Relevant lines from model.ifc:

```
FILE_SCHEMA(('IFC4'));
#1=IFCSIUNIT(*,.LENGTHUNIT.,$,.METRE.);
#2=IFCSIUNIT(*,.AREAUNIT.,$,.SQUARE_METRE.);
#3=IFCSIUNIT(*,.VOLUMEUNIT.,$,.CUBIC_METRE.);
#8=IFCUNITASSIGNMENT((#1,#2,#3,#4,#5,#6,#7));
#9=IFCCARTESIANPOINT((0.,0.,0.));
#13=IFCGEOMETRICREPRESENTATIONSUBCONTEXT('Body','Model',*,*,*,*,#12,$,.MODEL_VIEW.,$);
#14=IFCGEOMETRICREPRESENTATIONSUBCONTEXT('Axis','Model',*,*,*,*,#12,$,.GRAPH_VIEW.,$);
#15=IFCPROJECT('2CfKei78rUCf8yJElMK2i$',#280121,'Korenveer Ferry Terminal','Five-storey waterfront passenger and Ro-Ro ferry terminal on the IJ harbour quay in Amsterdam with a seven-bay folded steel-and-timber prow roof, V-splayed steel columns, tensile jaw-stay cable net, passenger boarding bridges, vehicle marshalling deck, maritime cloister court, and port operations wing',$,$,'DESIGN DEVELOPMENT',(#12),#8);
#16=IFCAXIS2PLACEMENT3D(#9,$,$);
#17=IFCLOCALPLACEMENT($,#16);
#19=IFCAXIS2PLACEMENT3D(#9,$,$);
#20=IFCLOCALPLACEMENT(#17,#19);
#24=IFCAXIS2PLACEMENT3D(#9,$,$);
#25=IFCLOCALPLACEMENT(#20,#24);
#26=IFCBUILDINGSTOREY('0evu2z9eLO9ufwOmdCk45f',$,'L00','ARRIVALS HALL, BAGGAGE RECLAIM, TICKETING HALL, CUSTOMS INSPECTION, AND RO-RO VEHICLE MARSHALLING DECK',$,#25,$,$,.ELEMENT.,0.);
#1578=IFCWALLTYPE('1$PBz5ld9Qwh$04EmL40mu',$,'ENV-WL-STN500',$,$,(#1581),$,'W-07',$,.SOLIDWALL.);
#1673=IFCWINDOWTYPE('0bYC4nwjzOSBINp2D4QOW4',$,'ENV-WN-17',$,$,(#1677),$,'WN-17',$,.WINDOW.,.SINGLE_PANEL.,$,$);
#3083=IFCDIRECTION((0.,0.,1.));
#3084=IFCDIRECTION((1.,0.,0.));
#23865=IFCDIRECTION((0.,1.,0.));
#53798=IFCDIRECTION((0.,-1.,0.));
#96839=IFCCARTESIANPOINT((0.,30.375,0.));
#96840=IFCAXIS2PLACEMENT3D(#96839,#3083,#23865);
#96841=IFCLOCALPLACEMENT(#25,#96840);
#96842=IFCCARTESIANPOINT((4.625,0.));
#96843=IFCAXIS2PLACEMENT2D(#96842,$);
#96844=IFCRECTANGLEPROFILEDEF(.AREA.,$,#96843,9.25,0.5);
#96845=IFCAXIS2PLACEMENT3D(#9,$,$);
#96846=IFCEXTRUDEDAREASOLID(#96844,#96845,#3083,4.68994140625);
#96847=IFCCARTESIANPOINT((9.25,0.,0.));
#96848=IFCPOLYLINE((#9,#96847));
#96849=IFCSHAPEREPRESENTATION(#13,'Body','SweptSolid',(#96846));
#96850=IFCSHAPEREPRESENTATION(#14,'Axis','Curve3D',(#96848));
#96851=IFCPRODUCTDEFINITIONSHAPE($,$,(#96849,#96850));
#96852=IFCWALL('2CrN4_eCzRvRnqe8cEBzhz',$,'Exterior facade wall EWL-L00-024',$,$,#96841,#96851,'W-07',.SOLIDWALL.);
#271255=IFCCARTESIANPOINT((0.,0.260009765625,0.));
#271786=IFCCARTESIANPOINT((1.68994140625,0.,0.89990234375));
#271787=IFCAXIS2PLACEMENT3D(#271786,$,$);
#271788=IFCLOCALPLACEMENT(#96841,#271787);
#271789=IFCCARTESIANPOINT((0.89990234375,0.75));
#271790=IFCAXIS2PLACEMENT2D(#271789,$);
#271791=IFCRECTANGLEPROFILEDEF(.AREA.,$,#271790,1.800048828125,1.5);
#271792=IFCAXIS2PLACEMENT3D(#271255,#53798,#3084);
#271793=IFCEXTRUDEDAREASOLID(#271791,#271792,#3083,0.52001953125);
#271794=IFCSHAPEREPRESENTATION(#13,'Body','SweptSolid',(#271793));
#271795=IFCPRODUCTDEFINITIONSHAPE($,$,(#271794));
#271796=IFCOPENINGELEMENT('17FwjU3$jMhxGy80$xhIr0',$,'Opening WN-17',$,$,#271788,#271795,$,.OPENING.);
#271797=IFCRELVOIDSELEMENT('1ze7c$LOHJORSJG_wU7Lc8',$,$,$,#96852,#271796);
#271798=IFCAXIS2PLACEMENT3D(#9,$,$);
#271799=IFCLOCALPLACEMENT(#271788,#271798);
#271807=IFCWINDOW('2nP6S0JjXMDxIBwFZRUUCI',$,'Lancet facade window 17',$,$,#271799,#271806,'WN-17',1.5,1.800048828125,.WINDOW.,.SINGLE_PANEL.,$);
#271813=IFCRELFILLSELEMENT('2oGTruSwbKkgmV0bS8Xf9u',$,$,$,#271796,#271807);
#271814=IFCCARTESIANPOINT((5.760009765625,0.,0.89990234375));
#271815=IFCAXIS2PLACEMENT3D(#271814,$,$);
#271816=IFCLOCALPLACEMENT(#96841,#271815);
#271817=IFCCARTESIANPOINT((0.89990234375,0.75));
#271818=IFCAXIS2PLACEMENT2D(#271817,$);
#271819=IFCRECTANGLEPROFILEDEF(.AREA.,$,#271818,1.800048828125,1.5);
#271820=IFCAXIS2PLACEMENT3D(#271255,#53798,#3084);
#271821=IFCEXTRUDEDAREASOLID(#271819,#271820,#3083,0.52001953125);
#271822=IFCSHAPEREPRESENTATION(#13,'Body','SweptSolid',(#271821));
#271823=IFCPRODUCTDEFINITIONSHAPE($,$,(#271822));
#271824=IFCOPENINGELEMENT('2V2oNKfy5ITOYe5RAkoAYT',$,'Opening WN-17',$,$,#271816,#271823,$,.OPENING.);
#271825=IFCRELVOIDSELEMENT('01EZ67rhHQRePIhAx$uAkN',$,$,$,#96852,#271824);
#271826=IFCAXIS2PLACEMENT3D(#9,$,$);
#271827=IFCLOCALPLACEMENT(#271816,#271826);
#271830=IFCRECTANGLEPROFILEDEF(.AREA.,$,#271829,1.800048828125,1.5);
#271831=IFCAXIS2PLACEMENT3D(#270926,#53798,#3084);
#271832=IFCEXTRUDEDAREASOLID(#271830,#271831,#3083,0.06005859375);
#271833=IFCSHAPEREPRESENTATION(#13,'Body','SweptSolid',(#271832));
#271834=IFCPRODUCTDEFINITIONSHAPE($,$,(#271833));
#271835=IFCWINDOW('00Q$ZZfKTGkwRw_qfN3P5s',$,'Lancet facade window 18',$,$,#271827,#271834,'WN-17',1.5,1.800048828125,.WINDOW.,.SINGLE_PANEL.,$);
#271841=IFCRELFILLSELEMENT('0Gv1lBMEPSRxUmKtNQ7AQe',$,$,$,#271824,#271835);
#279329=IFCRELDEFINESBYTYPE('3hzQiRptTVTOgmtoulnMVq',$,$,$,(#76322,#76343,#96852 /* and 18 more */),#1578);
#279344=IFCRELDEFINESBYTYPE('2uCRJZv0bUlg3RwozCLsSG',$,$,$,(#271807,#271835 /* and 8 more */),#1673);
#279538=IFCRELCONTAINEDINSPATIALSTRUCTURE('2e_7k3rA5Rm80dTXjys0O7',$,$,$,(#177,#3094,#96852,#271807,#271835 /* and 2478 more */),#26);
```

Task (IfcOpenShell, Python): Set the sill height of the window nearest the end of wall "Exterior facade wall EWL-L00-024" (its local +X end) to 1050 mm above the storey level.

```python
import numpy as np
import ifcopenshell
import ifcopenshell.api.geometry
import ifcopenshell.geom
import ifcopenshell.util.element
import ifcopenshell.util.placement
import ifcopenshell.util.shape
import ifcopenshell.util.unit

model = ifcopenshell.open("model.ifc")
unit_scale = ifcopenshell.util.unit.calculate_unit_scale(model)

window = model.by_guid("00Q$ZZfKTGkwRw_qfN3P5s")
opening = window.FillsVoids[0].RelatingOpeningElement
storey = ifcopenshell.util.element.get_container(window, ifc_class="IfcBuildingStorey")
level = ifcopenshell.util.placement.get_local_placement(storey.ObjectPlacement)[2, 3]

# The opening's origin need not be at the sill, so measure its lowest point.
shape = ifcopenshell.geom.create_shape(ifcopenshell.geom.settings(), opening)
bottom = ifcopenshell.util.shape.get_shape_bottom_elevation(shape, shape.geometry) / unit_scale
dz = level + 1.05 / unit_scale - bottom

shift = np.array([0.0, 0.0, dz])
# The window is placed relative to its opening, so it follows when the opening moves.
matrix = ifcopenshell.util.placement.get_local_placement(opening.ObjectPlacement)
matrix[:3, 3] += shift
ifcopenshell.api.geometry.edit_object_placement(
    model, product=opening, matrix=matrix, is_si=False, should_transform_children=True
)

print(f"moved by {dz * unit_scale:+.3f} m")

model.write("model_edited.ifc")
```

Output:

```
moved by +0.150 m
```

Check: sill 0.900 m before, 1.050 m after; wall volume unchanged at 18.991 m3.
